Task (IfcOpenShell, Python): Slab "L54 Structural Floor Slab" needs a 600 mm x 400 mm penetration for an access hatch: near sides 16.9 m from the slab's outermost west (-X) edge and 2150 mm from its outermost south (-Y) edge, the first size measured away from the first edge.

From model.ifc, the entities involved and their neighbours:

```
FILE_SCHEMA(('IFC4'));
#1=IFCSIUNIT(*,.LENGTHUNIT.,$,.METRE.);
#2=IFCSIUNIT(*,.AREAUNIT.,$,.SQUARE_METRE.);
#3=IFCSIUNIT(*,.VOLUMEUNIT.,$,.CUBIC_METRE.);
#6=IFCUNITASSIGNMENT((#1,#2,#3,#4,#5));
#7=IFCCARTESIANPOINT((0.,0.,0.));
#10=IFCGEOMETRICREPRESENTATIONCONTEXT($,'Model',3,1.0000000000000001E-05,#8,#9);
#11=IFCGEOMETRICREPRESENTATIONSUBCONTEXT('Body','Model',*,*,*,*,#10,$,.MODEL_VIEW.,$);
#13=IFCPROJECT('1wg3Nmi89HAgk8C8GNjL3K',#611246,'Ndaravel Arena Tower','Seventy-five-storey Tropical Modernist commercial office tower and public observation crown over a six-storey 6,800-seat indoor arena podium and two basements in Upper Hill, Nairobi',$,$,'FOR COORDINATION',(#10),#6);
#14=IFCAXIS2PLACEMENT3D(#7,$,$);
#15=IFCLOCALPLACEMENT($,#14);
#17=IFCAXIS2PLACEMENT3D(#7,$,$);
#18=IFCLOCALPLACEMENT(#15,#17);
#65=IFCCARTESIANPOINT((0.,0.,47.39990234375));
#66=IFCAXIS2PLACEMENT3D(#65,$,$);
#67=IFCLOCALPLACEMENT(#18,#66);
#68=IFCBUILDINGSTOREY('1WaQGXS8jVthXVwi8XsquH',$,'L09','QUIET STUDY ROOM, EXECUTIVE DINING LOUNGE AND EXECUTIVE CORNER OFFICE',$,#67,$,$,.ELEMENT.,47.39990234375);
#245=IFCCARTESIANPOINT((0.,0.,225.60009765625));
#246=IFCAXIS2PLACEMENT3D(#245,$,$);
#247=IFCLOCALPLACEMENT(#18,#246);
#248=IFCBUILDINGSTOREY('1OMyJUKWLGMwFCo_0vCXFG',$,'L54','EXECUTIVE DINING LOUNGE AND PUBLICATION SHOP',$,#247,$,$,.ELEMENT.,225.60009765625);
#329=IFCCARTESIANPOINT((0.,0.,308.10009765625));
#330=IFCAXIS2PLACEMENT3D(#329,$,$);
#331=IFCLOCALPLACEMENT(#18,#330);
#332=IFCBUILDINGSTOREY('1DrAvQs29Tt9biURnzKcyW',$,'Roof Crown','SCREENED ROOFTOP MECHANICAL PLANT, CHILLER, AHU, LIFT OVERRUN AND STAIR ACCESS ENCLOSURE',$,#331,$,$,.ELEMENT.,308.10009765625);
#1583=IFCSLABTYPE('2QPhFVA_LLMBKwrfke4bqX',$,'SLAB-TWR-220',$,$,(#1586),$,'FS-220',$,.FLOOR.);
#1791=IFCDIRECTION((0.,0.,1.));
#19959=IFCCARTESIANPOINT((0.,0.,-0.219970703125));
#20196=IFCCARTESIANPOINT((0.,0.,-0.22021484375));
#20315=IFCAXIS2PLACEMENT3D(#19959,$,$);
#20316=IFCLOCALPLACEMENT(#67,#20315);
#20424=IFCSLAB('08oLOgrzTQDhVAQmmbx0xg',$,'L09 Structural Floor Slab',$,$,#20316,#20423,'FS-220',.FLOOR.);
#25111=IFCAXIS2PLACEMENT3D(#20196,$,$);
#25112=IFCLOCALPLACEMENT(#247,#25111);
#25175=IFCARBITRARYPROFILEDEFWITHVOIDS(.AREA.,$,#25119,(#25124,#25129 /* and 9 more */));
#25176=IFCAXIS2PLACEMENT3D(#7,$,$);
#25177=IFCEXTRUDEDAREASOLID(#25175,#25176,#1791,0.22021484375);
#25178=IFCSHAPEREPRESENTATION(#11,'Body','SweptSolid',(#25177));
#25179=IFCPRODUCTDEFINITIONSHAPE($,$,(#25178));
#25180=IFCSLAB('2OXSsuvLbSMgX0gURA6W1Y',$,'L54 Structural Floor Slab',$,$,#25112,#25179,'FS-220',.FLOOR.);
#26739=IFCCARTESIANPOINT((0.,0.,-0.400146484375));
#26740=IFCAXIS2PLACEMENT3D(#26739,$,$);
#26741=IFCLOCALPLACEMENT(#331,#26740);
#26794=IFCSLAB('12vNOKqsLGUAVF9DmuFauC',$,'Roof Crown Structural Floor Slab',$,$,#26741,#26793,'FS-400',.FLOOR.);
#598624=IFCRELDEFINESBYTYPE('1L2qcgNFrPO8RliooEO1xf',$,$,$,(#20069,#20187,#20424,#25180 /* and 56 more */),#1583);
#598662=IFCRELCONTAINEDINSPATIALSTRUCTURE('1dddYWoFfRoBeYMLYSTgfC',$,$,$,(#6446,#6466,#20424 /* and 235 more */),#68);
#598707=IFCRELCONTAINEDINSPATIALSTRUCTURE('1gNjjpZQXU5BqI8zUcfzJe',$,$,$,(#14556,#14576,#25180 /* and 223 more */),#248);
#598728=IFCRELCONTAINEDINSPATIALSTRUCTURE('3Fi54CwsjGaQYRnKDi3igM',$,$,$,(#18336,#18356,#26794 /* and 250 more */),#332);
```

```python
import numpy as np
import ifcopenshell
import ifcopenshell.api.feature
import ifcopenshell.api.geometry
import ifcopenshell.api.root
import ifcopenshell.geom
import ifcopenshell.util.placement
import ifcopenshell.util.representation
import ifcopenshell.util.shape
import ifcopenshell.util.unit

model = ifcopenshell.open("model.ifc")
unit_scale = ifcopenshell.util.unit.calculate_unit_scale(model)
settings = ifcopenshell.geom.settings()


def volume(element):
    """Net volume in cubic metres, openings subtracted."""
    shape = ifcopenshell.geom.create_shape(settings, element)
    return ifcopenshell.util.shape.get_volume(shape.geometry)


slab = model.by_id(25180)
before = volume(slab)

# Extent in the slab's own axes, in metres. The edges named are its -X and -Y sides.
slab_shape = ifcopenshell.geom.create_shape(settings, slab)
vertices = ifcopenshell.util.shape.get_vertices(slab_shape.geometry)
x_min, y_min, bottom = vertices.min(axis=0)
top = vertices[:, 2].max()

opening = ifcopenshell.api.root.create_entity(model, ifc_class="IfcOpeningElement", name="Access hatch opening", predefined_type="OPENING")
context = ifcopenshell.util.representation.get_context(model, "Model", "Body", "MODEL_VIEW")
width, depth = 0.6, 0.4
outline = [(0.0, 0.0), (width, 0.0), (width, depth), (0.0, depth), (0.0, 0.0)]
# Overshoot both faces by 50 mm so the cut is clean.
shape = ifcopenshell.api.geometry.add_slab_representation(
    model, context=context, depth=top - bottom + 0.1, polyline=outline
)
ifcopenshell.api.geometry.assign_representation(model, product=opening, representation=shape)

matrix = ifcopenshell.util.placement.get_local_placement(slab.ObjectPlacement)
matrix[:, 3] = matrix @ np.append(np.array([x_min + 16.9, y_min + 2.15, bottom - 0.05]) / unit_scale, 1.0)
ifcopenshell.api.geometry.edit_object_placement(model, product=opening, matrix=matrix, is_si=False)
ifcopenshell.api.feature.add_feature(model, feature=opening, element=slab)

after = volume(slab)

print(f"slab volume {before:.3f} -> {after:.3f} m3")

model.write("model_edited.ifc")
```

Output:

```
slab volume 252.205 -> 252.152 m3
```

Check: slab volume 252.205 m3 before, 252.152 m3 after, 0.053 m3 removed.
